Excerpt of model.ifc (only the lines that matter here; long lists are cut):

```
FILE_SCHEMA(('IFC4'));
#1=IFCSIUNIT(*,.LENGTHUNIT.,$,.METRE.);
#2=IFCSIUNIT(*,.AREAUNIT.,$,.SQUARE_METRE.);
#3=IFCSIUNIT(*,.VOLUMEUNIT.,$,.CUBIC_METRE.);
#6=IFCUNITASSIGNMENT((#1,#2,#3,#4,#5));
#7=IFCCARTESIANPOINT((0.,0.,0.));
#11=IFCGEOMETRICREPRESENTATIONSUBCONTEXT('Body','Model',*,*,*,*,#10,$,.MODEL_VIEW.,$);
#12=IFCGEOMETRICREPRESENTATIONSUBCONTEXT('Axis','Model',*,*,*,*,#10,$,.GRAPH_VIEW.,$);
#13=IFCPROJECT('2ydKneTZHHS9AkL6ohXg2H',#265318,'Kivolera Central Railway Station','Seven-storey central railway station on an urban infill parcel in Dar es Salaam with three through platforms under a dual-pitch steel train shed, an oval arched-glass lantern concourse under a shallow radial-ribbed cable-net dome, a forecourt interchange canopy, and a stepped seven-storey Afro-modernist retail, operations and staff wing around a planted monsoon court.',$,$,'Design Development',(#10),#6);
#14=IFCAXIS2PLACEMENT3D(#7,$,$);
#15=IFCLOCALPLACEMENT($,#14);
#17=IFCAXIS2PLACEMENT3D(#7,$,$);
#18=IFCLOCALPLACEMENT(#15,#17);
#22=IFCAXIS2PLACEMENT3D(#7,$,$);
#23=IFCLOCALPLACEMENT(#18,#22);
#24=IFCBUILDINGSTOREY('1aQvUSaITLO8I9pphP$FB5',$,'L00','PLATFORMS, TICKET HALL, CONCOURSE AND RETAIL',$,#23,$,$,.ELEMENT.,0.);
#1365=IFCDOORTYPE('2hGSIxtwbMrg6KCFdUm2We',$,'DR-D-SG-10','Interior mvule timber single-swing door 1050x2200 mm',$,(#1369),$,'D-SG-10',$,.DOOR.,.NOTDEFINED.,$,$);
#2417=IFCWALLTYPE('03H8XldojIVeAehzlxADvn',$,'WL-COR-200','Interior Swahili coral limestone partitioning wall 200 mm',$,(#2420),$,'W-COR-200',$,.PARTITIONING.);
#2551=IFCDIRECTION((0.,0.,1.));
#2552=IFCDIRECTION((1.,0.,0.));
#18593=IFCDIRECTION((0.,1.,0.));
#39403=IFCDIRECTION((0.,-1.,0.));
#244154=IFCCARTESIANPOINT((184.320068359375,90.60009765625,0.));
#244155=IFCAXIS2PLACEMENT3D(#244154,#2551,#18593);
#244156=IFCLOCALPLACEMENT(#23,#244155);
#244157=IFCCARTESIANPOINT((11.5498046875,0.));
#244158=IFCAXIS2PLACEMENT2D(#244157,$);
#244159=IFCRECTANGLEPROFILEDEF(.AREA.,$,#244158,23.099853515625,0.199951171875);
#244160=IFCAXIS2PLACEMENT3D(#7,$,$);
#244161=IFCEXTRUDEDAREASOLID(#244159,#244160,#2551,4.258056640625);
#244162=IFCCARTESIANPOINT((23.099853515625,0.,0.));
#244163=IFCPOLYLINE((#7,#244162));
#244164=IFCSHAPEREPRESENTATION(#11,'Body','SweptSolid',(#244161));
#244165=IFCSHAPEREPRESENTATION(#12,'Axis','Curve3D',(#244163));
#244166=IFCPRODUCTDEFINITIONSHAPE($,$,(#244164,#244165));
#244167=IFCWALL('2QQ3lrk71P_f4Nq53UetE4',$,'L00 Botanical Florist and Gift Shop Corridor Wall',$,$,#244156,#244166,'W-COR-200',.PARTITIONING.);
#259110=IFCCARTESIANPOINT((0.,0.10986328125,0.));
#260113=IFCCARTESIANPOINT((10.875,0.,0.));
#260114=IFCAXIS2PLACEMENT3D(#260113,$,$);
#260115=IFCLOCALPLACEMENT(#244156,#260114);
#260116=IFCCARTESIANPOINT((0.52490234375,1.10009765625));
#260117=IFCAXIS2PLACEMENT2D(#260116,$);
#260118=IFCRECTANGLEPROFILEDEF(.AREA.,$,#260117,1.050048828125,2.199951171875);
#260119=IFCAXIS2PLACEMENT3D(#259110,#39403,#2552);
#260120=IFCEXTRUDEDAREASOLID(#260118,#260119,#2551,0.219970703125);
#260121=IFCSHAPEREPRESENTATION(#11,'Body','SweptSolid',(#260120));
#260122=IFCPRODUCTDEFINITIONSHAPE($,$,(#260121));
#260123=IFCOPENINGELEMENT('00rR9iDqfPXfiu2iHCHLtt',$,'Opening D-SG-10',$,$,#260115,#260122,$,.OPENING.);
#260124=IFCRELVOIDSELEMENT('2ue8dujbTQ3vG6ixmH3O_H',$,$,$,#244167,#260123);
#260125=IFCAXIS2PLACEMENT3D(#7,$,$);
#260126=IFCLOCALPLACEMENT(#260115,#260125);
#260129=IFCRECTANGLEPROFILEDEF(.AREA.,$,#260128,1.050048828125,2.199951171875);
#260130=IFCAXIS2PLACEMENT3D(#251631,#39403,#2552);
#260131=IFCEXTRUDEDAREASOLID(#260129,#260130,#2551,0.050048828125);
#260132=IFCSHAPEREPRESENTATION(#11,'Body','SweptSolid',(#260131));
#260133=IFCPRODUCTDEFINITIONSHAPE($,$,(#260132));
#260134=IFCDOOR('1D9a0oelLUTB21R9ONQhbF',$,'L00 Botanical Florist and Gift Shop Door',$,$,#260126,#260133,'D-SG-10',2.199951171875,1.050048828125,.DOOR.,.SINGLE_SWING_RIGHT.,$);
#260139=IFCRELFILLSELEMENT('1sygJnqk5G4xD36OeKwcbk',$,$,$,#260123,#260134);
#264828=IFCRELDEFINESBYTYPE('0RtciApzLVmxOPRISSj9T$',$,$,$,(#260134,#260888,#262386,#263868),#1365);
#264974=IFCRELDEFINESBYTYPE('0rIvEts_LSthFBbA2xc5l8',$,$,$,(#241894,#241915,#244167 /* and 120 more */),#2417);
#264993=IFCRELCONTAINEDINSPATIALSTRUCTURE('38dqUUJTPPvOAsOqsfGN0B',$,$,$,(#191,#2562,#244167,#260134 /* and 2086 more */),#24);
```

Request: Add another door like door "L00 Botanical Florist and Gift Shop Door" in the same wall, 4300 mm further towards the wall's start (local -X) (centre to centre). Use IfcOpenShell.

```python
import ifcopenshell
import ifcopenshell.api.feature
import ifcopenshell.api.geometry
import ifcopenshell.api.root
import ifcopenshell.geom
import ifcopenshell.util.element
import ifcopenshell.util.placement
import ifcopenshell.util.shape
import ifcopenshell.util.unit

model = ifcopenshell.open("model.ifc")
unit_scale = ifcopenshell.util.unit.calculate_unit_scale(model)
settings = ifcopenshell.geom.settings()


def volume(element):
    """Net volume in cubic metres, openings subtracted."""
    shape = ifcopenshell.geom.create_shape(settings, element)
    return ifcopenshell.util.shape.get_volume(shape.geometry)


door = model.by_guid("1D9a0oelLUTB21R9ONQhbF")
opening = door.FillsVoids[0].RelatingOpeningElement
wall = opening.VoidsElements[0].RelatingBuildingElement
before = volume(wall)
shift = ifcopenshell.util.placement.get_local_placement(wall.ObjectPlacement)[:3, 0] * -4.3 / unit_scale

# copy_class copies the void relationship, type, container and properties, but no geometry.
new_opening = ifcopenshell.api.root.copy_class(model, product=opening)
new_opening.Representation = ifcopenshell.util.element.copy_deep(
    model, opening.Representation, exclude=["IfcGeometricRepresentationContext", "IfcRepresentationMap"]
)
new_door = ifcopenshell.api.root.copy_class(model, product=door)
new_door.Representation = ifcopenshell.util.element.copy_deep(
    model, door.Representation, exclude=["IfcGeometricRepresentationContext", "IfcRepresentationMap"]
)
new_door.Tag = None
ifcopenshell.api.feature.add_filling(model, opening=new_opening, element=new_door)

for old, new in ((opening, new_opening), (door, new_door)):
    matrix = ifcopenshell.util.placement.get_local_placement(old.ObjectPlacement)
    matrix[:3, 3] += shift
    ifcopenshell.api.geometry.edit_object_placement(model, product=new, matrix=matrix, is_si=False)

after = volume(wall)

print(f"wall volume {before:.3f} -> {after:.3f} m3")

model.write("model_v2.ifc")
```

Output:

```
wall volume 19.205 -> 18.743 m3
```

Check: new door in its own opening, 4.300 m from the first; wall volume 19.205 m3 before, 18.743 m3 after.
